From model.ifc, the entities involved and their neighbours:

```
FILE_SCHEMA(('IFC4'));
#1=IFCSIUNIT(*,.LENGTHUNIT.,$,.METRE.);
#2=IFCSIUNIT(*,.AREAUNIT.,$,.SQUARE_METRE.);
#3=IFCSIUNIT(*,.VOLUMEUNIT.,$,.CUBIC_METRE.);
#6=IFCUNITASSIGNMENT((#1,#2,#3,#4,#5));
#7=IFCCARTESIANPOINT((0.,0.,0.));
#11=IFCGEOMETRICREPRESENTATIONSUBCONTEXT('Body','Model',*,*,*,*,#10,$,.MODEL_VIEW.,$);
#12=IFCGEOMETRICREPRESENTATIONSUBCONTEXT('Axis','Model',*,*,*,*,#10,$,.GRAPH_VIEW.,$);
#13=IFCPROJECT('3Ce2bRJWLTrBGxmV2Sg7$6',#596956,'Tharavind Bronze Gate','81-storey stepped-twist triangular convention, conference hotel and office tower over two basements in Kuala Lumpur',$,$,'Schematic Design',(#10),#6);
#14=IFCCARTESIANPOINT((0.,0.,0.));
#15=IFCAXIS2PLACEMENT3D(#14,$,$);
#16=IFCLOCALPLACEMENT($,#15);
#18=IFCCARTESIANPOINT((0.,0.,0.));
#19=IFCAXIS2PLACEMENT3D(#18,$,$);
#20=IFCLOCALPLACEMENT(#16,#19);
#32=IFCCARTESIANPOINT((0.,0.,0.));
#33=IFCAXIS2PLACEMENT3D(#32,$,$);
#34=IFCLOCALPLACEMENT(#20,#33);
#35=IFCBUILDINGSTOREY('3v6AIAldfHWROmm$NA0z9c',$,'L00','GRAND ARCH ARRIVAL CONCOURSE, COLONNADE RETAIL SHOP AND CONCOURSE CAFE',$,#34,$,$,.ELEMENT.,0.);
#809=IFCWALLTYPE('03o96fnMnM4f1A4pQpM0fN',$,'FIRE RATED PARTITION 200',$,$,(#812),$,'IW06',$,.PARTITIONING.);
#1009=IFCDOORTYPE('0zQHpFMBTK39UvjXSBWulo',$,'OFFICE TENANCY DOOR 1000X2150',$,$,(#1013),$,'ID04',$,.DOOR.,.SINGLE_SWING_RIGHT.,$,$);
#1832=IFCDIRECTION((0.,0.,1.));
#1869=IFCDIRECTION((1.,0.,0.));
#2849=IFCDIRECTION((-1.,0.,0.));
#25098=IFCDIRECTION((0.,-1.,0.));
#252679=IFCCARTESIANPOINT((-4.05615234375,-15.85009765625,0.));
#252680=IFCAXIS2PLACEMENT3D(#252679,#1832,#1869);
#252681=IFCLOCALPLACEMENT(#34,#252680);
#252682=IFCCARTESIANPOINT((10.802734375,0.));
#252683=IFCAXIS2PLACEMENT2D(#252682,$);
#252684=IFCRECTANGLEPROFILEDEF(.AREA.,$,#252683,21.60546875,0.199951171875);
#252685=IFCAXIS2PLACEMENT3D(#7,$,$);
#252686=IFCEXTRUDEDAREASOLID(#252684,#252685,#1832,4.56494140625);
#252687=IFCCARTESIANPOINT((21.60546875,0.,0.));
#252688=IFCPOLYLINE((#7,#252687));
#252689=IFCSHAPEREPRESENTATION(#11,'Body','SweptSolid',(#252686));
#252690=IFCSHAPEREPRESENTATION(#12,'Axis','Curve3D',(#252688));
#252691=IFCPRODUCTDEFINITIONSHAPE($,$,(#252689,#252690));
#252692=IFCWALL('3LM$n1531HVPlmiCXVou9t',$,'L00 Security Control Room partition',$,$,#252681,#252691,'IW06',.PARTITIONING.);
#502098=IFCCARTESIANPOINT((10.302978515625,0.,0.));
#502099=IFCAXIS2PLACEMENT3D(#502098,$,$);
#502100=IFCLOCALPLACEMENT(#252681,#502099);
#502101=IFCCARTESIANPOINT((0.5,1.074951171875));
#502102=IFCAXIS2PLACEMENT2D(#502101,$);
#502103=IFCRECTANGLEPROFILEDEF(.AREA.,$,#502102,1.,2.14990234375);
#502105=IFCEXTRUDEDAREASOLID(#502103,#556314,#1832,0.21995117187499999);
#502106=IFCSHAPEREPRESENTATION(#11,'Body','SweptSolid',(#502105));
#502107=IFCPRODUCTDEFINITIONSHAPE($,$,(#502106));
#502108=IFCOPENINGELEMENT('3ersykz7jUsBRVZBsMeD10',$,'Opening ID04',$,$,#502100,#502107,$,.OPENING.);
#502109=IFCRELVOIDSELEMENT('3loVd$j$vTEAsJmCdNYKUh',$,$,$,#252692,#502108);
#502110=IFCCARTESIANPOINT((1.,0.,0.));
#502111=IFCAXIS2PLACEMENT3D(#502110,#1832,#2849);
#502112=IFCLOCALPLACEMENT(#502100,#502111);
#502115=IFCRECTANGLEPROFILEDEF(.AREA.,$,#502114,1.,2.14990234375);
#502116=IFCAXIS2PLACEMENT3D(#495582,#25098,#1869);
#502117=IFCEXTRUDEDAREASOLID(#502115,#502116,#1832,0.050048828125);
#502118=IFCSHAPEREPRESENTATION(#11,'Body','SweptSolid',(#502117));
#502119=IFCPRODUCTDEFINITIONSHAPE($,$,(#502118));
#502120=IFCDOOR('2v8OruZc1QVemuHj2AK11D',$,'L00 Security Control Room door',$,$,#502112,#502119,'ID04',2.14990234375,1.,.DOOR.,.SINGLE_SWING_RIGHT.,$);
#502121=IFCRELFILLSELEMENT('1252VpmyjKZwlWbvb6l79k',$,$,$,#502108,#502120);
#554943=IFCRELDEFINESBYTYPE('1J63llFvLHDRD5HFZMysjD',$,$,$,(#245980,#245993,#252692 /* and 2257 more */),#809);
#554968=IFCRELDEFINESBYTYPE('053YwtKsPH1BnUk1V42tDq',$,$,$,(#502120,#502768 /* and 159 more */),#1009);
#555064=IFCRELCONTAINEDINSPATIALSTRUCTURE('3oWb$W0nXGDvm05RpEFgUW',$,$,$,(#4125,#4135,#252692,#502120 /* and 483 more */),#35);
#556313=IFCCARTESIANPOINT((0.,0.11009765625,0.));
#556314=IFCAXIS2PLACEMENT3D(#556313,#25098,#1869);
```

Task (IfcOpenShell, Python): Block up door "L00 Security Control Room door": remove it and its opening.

```python
import ifcopenshell
import ifcopenshell.api.feature
import ifcopenshell.api.root
import ifcopenshell.geom
import ifcopenshell.util.shape

model = ifcopenshell.open("model.ifc")
settings = ifcopenshell.geom.settings()


def volume(element):
    """Net volume in cubic metres, openings subtracted."""
    shape = ifcopenshell.geom.create_shape(settings, element)
    return ifcopenshell.util.shape.get_volume(shape.geometry)


door = model.by_guid("2v8OruZc1QVemuHj2AK11D")
opening = door.FillsVoids[0].RelatingOpeningElement
wall = opening.VoidsElements[0].RelatingBuildingElement
before = volume(wall)

ifcopenshell.api.root.remove_product(model, product=door)
ifcopenshell.api.feature.remove_feature(model, feature=opening)

after = volume(wall)

print(f"wall volume {before:.3f} -> {after:.3f} m3")

model.write("model_v2.ifc")
```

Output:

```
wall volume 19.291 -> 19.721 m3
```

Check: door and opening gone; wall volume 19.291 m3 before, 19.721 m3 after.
